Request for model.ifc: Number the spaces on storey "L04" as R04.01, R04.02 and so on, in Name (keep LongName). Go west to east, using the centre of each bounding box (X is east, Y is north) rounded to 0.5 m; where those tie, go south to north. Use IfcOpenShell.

First a look at what the model holds.

```python
import ifcopenshell
import ifcopenshell.util.element
import ifcopenshell.util.placement

model = ifcopenshell.open("model.ifc")
print(model.schema)
storey = next(s for s in model.by_type("IfcBuildingStorey") if s.Name == "L04")
spaces = [e for e in ifcopenshell.util.element.get_decomposition(storey) if e.is_a("IfcSpace")]
for e in sorted(spaces, key=lambda e: e.id()):
    origin = ifcopenshell.util.placement.get_local_placement(e.ObjectPlacement)[:3, 3]
    print(e.id(), e.Name, e.LongName, origin.round(2) + 0.0, sep=" | ")
```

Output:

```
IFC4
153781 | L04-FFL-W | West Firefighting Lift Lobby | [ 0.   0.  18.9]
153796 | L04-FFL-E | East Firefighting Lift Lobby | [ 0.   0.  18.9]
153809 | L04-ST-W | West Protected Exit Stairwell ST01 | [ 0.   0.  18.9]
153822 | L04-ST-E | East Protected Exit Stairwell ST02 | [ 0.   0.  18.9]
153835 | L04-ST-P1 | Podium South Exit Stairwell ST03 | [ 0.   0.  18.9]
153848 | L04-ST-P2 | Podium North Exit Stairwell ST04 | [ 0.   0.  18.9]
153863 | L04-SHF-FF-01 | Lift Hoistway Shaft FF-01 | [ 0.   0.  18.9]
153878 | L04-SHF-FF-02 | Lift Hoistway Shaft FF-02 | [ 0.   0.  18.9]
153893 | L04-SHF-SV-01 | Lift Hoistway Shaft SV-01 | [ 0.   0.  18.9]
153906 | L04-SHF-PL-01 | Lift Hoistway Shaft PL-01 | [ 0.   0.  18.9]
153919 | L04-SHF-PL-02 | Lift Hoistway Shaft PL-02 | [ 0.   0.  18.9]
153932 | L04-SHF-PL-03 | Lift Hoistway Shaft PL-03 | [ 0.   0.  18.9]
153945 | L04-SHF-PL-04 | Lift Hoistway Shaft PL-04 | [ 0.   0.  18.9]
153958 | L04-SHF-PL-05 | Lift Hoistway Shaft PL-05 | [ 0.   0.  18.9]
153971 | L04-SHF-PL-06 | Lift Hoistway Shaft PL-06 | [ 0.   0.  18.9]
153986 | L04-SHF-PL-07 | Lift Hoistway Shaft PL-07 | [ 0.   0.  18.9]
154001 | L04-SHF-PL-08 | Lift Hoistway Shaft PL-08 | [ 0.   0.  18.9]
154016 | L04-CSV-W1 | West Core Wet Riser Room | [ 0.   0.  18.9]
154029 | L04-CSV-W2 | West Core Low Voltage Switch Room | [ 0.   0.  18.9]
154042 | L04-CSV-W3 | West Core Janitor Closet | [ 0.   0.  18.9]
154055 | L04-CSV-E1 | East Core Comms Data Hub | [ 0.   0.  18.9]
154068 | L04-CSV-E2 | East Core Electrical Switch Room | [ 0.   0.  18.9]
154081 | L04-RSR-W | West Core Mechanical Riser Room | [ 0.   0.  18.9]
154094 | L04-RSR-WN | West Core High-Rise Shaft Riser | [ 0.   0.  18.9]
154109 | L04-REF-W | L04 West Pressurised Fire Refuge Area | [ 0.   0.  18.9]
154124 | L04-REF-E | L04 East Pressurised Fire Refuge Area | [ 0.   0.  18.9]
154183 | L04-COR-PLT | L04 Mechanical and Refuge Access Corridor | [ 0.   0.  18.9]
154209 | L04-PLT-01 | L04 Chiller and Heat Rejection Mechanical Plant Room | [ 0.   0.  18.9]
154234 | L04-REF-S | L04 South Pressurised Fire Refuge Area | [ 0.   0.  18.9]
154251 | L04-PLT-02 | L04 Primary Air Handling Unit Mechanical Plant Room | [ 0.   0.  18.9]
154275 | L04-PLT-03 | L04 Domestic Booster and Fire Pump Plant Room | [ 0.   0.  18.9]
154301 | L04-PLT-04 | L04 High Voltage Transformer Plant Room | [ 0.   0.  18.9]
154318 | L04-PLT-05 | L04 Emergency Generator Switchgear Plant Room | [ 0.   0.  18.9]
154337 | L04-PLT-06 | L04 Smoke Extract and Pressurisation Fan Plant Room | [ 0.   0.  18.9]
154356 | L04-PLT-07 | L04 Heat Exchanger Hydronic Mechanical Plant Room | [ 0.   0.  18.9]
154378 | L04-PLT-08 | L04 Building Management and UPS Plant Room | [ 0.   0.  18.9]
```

```python
import ifcopenshell
import ifcopenshell.geom
import ifcopenshell.util.element
import ifcopenshell.util.shape

model = ifcopenshell.open("model.ifc")
settings = ifcopenshell.geom.settings()
settings.set("use-world-coords", True)


def centre(element):
    shape = ifcopenshell.geom.create_shape(settings, element)
    return ifcopenshell.util.shape.get_bbox_centroid(shape.geometry)


storey = next(s for s in model.by_type("IfcBuildingStorey") if s.Name == "L04")
spaces = [e for e in ifcopenshell.util.element.get_decomposition(storey) if e.is_a("IfcSpace")]

# Insertion points can sit at a corner or the storey origin, so sort by the geometry (in metres).
centres = {e: centre(e) for e in spaces}
spaces.sort(key=lambda e: (round(centres[e][0] / 0.5), centres[e][1]))

for i, e in enumerate(spaces, start=1):
    number = f"R04.{i:02d}"
    e.Name = number
    print(e.id(), number)

model.write("model-out.ifc")
```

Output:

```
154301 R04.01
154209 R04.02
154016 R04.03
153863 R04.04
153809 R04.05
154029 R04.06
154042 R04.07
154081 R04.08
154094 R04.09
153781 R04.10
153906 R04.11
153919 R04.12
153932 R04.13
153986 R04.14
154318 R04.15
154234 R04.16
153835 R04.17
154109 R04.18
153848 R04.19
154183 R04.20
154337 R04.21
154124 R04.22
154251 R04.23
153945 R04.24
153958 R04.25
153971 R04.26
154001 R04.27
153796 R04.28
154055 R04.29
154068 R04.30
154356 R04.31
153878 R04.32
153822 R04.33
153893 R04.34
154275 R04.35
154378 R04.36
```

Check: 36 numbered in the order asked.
